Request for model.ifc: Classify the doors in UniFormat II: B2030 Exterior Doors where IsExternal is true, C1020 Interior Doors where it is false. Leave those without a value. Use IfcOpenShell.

First a look at what the model holds.

```python
import ifcopenshell
import ifcopenshell.util.element

model = ifcopenshell.open("model.ifc")
print(model.schema)
print("classifications:", [c.Name for c in model.by_type("IfcClassification")])
values = [ifcopenshell.util.element.get_pset(e, "Pset_DoorCommon", "IsExternal") for e in model.by_type("IfcDoor")]
for value in (True, False, None):
    print("IsExternal", value, values.count(value))
```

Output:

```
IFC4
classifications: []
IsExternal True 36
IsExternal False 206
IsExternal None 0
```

```python
import ifcopenshell
import ifcopenshell.api.classification
import ifcopenshell.util.element

model = ifcopenshell.open("model.ifc")

system = ifcopenshell.api.classification.add_classification(model, classification="UniFormat II")

doors = model.by_type("IfcDoor")
external = {e: ifcopenshell.util.element.get_pset(e, "Pset_DoorCommon", "IsExternal") for e in doors}
for flag, code, name in ((True, "B2030", "Exterior Doors"), (False, "C1020", "Interior Doors")):
    products = [e for e in doors if external[e] is flag]
    ifcopenshell.api.classification.add_reference(
        model, products=products, classification=system, identification=code, name=name
    )
    print(code, len(products))

model.write("model_v2.ifc")
```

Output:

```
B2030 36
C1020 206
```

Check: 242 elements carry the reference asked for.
